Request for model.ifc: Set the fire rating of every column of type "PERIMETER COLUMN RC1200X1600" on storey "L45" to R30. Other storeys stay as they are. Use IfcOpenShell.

First a look at what the model holds.

```python
import ifcopenshell
import ifcopenshell.util.element

model = ifcopenshell.open("model.ifc")
print(model.schema)
storey = next(s for s in model.by_type("IfcBuildingStorey") if s.Name == "L45")
columns = [e for e in ifcopenshell.util.element.get_decomposition(storey) if e.is_a("IfcColumn")]
seen = {}
for e in columns:
    element_type = ifcopenshell.util.element.get_type(e)
    key = (element_type.Name if element_type != e and element_type else None, ifcopenshell.util.element.get_pset(e, "Pset_ColumnCommon", "FireRating"))
    seen[key] = seen.get(key, 0) + 1
for (name, value), count in sorted(seen.items(), key=str):
    print(count, "x", name, "|", value)
```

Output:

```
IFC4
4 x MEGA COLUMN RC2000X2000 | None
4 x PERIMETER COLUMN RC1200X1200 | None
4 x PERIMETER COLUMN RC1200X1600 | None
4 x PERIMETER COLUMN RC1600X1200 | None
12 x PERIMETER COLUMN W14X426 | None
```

```python
import ifcopenshell
import ifcopenshell.api.pset
import ifcopenshell.util.element

model = ifcopenshell.open("model.ifc")

storey = next(s for s in model.by_type("IfcBuildingStorey") if s.Name == "L45")
columns = [e for e in ifcopenshell.util.element.get_decomposition(storey) if e.is_a("IfcColumn")]

count = 0
for e in columns:
    element_type = ifcopenshell.util.element.get_type(e)
    if element_type in (None, e) or element_type.Name != "PERIMETER COLUMN RC1200X1600":
        continue
    found = ifcopenshell.util.element.get_pset(e, "Pset_ColumnCommon", should_inherit=False)
    if found:
        pset = model.by_id(found["id"])
        if len(ifcopenshell.util.element.get_elements_by_pset(pset)) > 1:
            pset = ifcopenshell.api.pset.unshare_pset(model, products=[e], pset=pset)[0]
    else:
        pset = ifcopenshell.api.pset.add_pset(model, product=e, name="Pset_ColumnCommon")
    ifcopenshell.api.pset.edit_pset(model, pset=pset, properties={"FireRating": "R30"})
    count += 1

print(count, "columns updated")

model.write("model_rev.ifc")
```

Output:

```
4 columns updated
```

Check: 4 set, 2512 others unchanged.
